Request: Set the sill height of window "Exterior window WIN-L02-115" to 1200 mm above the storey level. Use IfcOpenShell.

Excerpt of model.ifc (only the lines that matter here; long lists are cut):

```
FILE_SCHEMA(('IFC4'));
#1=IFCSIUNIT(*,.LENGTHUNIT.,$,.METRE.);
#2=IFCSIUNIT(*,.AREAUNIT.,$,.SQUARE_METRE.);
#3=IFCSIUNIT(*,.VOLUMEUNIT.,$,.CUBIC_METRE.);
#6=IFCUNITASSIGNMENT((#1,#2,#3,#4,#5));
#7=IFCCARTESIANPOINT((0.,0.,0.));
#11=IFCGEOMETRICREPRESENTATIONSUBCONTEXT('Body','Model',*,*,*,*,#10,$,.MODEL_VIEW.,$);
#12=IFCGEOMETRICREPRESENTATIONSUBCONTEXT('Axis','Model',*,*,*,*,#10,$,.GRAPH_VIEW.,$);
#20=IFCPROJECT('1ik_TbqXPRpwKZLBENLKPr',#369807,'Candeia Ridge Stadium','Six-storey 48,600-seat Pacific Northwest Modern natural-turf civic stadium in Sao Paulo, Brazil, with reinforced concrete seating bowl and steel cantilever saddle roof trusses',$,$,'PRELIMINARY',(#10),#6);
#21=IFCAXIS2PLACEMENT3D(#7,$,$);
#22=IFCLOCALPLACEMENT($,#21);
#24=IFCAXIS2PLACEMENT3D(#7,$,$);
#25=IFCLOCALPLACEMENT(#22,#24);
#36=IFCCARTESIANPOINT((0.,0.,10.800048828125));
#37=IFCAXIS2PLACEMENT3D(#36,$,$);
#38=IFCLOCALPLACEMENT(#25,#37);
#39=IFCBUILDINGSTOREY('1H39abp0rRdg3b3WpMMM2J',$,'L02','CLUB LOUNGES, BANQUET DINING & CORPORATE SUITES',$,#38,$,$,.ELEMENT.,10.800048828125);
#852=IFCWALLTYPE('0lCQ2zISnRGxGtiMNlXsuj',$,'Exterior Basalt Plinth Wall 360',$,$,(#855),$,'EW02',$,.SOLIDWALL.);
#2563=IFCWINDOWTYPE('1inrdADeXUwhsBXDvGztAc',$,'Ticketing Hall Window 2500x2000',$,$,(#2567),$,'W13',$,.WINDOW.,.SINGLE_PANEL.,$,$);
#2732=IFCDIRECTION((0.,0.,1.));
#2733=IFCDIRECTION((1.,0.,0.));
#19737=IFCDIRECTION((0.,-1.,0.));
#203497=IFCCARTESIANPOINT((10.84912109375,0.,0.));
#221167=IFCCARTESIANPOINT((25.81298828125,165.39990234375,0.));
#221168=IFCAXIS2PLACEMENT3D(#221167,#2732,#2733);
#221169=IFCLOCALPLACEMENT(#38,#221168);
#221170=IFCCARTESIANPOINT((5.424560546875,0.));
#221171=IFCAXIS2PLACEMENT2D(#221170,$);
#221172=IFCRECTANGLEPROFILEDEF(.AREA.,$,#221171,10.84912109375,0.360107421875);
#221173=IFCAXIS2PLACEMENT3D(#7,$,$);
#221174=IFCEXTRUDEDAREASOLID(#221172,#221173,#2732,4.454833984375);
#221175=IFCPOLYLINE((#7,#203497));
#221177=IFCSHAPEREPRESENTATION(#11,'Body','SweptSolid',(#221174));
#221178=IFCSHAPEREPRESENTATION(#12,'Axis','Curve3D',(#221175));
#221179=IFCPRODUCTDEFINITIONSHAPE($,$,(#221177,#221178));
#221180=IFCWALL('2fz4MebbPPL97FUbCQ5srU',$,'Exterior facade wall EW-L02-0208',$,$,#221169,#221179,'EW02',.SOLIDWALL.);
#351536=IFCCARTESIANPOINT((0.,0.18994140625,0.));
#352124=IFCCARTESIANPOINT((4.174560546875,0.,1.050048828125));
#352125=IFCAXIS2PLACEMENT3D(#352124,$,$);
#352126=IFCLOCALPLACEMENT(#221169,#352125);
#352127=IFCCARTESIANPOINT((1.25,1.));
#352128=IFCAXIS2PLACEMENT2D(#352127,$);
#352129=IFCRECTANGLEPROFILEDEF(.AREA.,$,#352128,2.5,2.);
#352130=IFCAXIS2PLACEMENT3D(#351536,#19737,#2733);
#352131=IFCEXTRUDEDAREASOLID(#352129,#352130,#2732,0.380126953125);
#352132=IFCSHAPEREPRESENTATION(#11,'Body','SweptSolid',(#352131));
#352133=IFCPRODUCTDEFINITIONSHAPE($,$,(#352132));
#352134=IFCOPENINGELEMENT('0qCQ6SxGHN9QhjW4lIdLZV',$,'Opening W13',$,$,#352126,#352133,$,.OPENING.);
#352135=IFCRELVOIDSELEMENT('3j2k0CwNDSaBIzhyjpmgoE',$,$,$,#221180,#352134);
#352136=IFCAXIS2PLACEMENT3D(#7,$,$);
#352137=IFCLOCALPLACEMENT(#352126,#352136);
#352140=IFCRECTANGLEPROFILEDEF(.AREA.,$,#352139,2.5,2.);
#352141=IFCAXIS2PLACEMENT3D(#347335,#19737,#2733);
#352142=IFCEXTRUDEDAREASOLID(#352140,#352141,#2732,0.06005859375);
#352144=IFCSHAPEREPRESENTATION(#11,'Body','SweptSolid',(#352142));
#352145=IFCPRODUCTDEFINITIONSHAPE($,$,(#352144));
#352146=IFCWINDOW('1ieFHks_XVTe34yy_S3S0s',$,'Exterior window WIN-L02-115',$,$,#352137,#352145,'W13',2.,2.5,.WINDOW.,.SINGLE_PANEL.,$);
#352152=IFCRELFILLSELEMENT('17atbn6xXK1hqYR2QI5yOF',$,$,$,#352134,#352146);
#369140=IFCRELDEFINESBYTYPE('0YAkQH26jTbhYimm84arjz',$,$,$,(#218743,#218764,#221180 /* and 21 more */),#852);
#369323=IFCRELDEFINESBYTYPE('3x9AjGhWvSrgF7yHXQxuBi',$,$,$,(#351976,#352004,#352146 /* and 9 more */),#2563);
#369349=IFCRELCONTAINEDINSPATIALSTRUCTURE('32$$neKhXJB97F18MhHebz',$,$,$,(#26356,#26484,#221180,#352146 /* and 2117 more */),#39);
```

```python
import numpy as np
import ifcopenshell
import ifcopenshell.api.geometry
import ifcopenshell.geom
import ifcopenshell.util.element
import ifcopenshell.util.placement
import ifcopenshell.util.shape
import ifcopenshell.util.unit

model = ifcopenshell.open("model.ifc")
unit_scale = ifcopenshell.util.unit.calculate_unit_scale(model)

window = model.by_guid("1ieFHks_XVTe34yy_S3S0s")
opening = window.FillsVoids[0].RelatingOpeningElement
storey = ifcopenshell.util.element.get_container(window, ifc_class="IfcBuildingStorey")
level = ifcopenshell.util.placement.get_local_placement(storey.ObjectPlacement)[2, 3]

# The opening's origin need not be at the sill, so measure its lowest point.
shape = ifcopenshell.geom.create_shape(ifcopenshell.geom.settings(), opening)
bottom = ifcopenshell.util.shape.get_shape_bottom_elevation(shape, shape.geometry) / unit_scale
dz = level + 1.2 / unit_scale - bottom

shift = np.array([0.0, 0.0, dz])
# The window is placed relative to its opening, so it follows when the opening moves.
matrix = ifcopenshell.util.placement.get_local_placement(opening.ObjectPlacement)
matrix[:3, 3] += shift
ifcopenshell.api.geometry.edit_object_placement(
    model, product=opening, matrix=matrix, is_si=False, should_transform_children=True
)

print(f"moved by {dz * unit_scale:+.3f} m")

model.write("model_updated.ifc")
```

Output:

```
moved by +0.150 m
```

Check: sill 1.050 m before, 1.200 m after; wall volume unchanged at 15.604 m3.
